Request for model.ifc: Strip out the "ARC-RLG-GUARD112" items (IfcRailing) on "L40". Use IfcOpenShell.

First a look at what the model holds.

```python
import ifcopenshell
import ifcopenshell.util.element

model = ifcopenshell.open("model.ifc")
print(model.schema)
storey = next(s for s in model.by_type("IfcBuildingStorey") if s.Name == "L40")
railings = [e for e in ifcopenshell.util.element.get_decomposition(storey) if e.is_a("IfcRailing")]
seen = {}
for e in railings:
    element_type = ifcopenshell.util.element.get_type(e)
    name = element_type.Name if element_type not in (None, e) else None
    seen[name] = seen.get(name, 0) + 1
for name, count in sorted(seen.items(), key=str):
    print(count, "x", name)
```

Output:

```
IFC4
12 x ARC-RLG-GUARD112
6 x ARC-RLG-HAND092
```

```python
import ifcopenshell
import ifcopenshell.api.root
import ifcopenshell.util.element

model = ifcopenshell.open("model.ifc")

storey = next(s for s in model.by_type("IfcBuildingStorey") if s.Name == "L40")
railings = [e for e in ifcopenshell.util.element.get_decomposition(storey) if e.is_a("IfcRailing")]
targets = [e for e in railings if (t := ifcopenshell.util.element.get_type(e)) not in (None, e) and t.Name == "ARC-RLG-GUARD112"]

for e in targets:
    ifcopenshell.api.root.remove_product(model, product=e)
print(len(targets), "removed")

model.write("model_updated.ifc")
```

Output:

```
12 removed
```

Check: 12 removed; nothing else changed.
